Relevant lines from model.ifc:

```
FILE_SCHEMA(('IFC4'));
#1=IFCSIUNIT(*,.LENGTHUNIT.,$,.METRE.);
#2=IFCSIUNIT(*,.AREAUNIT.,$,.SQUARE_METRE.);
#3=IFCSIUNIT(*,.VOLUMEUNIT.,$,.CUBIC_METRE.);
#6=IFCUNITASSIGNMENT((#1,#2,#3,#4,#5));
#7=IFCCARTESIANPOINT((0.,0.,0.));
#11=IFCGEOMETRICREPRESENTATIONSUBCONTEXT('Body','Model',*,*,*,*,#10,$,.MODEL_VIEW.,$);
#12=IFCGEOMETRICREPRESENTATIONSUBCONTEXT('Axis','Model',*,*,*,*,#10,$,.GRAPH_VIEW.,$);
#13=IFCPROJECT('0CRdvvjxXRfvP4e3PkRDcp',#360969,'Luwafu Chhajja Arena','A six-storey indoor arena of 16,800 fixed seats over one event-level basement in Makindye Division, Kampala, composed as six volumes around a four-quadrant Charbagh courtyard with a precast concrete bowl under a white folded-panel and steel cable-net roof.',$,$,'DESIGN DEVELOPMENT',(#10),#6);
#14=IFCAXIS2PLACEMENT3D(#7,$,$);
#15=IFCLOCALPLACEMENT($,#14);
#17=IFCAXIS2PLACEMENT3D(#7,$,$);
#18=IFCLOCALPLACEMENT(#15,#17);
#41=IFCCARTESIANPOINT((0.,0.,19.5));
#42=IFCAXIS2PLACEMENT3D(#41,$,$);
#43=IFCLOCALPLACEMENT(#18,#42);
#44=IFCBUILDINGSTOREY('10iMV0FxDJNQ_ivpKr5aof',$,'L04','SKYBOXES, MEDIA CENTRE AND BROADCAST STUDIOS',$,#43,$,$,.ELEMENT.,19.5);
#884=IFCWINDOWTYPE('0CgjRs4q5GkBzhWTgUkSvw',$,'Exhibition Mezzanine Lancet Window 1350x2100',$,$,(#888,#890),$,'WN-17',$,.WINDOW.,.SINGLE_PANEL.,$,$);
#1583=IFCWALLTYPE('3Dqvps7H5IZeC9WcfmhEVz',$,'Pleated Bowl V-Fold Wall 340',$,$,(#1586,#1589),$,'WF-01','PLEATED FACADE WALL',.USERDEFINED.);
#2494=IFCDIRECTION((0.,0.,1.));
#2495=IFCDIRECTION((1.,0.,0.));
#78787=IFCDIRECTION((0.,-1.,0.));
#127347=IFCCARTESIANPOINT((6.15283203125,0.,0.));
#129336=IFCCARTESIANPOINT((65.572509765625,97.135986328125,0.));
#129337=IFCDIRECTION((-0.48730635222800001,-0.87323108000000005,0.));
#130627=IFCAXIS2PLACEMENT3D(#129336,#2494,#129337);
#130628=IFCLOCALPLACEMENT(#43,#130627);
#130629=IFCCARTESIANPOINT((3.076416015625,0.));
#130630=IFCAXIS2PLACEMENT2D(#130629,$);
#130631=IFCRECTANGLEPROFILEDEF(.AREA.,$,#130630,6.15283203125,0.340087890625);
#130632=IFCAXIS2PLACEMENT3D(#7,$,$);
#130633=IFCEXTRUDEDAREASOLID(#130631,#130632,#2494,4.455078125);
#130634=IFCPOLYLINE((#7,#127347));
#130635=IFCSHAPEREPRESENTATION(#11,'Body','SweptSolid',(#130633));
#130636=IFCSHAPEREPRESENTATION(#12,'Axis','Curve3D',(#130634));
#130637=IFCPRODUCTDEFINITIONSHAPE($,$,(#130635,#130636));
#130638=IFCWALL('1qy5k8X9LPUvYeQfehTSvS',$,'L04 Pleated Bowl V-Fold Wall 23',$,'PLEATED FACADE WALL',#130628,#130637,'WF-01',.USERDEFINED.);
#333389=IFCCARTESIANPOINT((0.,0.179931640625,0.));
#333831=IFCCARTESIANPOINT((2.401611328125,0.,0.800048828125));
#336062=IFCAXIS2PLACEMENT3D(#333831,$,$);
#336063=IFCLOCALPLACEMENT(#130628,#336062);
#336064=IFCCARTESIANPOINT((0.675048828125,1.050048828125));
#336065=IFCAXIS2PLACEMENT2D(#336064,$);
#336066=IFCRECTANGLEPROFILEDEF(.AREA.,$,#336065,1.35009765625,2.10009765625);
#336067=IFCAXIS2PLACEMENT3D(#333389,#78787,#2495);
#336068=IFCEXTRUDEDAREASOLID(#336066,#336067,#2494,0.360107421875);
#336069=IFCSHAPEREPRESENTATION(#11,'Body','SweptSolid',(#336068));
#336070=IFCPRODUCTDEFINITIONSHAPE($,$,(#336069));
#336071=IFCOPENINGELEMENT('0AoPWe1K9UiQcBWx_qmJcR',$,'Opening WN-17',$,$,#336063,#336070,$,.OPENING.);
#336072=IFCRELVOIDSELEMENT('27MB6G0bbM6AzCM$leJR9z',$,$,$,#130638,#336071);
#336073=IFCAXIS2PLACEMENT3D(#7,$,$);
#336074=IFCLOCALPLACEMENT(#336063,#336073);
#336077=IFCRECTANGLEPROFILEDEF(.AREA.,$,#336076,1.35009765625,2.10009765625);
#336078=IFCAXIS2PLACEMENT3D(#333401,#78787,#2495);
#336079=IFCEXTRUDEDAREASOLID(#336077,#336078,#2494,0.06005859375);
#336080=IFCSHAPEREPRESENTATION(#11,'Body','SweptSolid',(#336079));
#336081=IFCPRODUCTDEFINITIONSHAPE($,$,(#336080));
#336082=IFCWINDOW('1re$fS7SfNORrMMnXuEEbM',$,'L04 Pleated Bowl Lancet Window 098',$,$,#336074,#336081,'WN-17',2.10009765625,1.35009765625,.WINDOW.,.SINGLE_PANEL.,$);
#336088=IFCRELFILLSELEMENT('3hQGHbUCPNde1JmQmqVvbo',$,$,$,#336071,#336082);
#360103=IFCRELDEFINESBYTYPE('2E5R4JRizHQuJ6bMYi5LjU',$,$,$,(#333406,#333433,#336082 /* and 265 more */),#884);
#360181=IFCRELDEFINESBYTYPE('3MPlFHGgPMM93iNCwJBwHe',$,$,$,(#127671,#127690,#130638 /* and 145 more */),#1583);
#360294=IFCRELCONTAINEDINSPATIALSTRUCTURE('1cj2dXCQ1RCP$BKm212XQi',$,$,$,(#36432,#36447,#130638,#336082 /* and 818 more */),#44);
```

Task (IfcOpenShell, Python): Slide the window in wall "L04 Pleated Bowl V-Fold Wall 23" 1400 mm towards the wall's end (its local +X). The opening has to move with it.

```python
import ifcopenshell
import ifcopenshell.api.geometry
import ifcopenshell.util.placement
import ifcopenshell.util.unit

model = ifcopenshell.open("model.ifc")
unit_scale = ifcopenshell.util.unit.calculate_unit_scale(model)

window = model.by_guid("1re$fS7SfNORrMMnXuEEbM")
opening = window.FillsVoids[0].RelatingOpeningElement
wall = opening.VoidsElements[0].RelatingBuildingElement

wall_matrix = ifcopenshell.util.placement.get_local_placement(wall.ObjectPlacement)
shift = wall_matrix[:3, 0] * 1.4 / unit_scale
before = ifcopenshell.util.placement.get_local_placement(window.ObjectPlacement)[:3, 3].copy()

# The window is placed relative to its opening, so it follows when the opening moves.
matrix = ifcopenshell.util.placement.get_local_placement(opening.ObjectPlacement)
matrix[:3, 3] += shift
ifcopenshell.api.geometry.edit_object_placement(
    model, product=opening, matrix=matrix, is_si=False, should_transform_children=True
)

after = ifcopenshell.util.placement.get_local_placement(window.ObjectPlacement)[:3, 3]
print("window moved by", (after - before).round(3) + 0.0)

model.write("model-out.ifc")
```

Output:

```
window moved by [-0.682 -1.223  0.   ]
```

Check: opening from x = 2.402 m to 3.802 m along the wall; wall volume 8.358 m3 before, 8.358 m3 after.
